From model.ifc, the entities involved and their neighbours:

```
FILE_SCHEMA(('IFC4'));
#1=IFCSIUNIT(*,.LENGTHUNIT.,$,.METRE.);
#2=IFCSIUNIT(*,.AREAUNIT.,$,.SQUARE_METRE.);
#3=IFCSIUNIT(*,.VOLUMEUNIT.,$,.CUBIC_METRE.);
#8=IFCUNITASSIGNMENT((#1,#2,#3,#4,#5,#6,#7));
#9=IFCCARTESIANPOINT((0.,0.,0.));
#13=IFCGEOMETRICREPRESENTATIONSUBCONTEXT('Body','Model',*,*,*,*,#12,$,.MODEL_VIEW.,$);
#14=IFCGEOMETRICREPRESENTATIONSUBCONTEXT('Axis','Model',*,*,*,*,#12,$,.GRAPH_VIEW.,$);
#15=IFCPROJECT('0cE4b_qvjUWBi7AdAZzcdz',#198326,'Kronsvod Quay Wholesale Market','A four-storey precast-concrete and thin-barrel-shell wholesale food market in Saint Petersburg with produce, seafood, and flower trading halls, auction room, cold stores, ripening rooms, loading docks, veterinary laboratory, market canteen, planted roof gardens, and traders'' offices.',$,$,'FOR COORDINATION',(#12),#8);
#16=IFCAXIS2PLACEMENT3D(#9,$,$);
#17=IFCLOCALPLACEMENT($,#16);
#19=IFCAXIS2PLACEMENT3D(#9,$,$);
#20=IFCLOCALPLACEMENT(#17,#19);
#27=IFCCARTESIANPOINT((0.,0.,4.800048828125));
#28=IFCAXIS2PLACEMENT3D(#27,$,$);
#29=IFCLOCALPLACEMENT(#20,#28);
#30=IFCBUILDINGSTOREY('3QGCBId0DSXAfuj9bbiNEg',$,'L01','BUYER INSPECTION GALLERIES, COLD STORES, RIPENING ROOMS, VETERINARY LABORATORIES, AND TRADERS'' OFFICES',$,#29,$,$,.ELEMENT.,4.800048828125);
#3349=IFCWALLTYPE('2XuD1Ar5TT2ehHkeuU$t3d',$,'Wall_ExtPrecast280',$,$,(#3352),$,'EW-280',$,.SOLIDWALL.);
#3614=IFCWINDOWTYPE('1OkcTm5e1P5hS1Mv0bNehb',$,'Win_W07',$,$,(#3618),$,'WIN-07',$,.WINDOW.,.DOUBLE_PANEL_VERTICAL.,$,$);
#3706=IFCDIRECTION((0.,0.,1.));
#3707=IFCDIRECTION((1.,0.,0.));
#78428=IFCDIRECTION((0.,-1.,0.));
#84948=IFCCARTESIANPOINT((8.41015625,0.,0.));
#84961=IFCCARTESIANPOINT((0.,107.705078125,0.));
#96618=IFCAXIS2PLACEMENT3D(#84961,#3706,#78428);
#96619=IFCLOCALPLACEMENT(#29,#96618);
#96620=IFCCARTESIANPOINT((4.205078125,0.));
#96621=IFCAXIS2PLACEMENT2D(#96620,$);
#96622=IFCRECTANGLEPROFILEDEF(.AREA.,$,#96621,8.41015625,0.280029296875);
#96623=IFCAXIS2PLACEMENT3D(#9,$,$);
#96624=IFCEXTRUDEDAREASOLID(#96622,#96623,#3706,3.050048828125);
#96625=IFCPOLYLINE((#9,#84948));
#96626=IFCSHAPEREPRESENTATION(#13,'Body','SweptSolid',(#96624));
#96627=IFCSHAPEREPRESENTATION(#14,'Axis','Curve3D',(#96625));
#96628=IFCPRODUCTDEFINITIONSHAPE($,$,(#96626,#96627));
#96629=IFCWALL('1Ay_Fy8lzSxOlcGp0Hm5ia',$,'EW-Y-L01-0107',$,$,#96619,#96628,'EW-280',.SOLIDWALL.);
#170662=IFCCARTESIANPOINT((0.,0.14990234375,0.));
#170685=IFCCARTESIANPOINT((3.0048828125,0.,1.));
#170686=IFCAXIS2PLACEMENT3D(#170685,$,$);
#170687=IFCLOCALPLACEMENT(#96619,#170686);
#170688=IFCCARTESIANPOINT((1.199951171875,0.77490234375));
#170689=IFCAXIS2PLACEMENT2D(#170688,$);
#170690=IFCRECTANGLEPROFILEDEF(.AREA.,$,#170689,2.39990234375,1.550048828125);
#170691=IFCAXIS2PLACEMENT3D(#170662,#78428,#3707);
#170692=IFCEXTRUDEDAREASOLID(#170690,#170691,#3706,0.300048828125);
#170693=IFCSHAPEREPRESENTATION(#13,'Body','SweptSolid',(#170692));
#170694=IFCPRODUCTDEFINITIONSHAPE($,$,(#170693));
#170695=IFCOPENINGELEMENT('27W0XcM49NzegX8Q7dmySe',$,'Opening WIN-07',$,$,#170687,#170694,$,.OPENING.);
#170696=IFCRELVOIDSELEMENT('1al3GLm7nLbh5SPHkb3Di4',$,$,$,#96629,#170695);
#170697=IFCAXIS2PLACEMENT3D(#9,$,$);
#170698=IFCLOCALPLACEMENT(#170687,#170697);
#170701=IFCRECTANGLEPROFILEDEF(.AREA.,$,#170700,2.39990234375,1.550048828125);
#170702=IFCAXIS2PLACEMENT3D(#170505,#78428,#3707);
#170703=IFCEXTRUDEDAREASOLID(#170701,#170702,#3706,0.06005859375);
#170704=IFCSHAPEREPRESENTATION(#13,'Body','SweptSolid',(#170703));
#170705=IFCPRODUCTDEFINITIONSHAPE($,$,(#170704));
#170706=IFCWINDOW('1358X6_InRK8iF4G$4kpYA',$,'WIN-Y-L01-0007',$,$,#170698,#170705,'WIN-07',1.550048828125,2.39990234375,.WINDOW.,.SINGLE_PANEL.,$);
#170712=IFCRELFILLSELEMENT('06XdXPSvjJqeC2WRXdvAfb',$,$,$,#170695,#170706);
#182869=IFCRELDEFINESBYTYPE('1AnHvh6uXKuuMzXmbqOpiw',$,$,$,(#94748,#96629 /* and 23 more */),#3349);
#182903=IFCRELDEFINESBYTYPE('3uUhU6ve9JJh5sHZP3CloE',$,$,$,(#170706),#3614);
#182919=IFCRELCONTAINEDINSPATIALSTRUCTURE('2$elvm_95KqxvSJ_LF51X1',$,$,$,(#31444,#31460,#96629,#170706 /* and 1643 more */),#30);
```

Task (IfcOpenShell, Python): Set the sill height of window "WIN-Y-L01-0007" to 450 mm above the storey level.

```python
import numpy as np
import ifcopenshell
import ifcopenshell.api.geometry
import ifcopenshell.geom
import ifcopenshell.util.element
import ifcopenshell.util.placement
import ifcopenshell.util.shape
import ifcopenshell.util.unit

model = ifcopenshell.open("model.ifc")
unit_scale = ifcopenshell.util.unit.calculate_unit_scale(model)

window = model.by_id(170706)
opening = window.FillsVoids[0].RelatingOpeningElement
storey = ifcopenshell.util.element.get_container(window, ifc_class="IfcBuildingStorey")
level = ifcopenshell.util.placement.get_local_placement(storey.ObjectPlacement)[2, 3]

# The opening's origin need not be at the sill, so measure its lowest point.
shape = ifcopenshell.geom.create_shape(ifcopenshell.geom.settings(), opening)
bottom = ifcopenshell.util.shape.get_shape_bottom_elevation(shape, shape.geometry) / unit_scale
dz = level + 0.45 - bottom

shift = np.array([0.0, 0.0, dz])
# The window is placed relative to its opening, so it follows when the opening moves.
matrix = ifcopenshell.util.placement.get_local_placement(opening.ObjectPlacement)
matrix[:3, 3] += shift
ifcopenshell.api.geometry.edit_object_placement(
    model, product=opening, matrix=matrix, is_si=False, should_transform_children=True
)

print(f"moved by {dz * unit_scale:+.3f} m")

model.write("model-out.ifc")
```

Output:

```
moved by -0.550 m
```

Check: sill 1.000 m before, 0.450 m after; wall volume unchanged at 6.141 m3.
